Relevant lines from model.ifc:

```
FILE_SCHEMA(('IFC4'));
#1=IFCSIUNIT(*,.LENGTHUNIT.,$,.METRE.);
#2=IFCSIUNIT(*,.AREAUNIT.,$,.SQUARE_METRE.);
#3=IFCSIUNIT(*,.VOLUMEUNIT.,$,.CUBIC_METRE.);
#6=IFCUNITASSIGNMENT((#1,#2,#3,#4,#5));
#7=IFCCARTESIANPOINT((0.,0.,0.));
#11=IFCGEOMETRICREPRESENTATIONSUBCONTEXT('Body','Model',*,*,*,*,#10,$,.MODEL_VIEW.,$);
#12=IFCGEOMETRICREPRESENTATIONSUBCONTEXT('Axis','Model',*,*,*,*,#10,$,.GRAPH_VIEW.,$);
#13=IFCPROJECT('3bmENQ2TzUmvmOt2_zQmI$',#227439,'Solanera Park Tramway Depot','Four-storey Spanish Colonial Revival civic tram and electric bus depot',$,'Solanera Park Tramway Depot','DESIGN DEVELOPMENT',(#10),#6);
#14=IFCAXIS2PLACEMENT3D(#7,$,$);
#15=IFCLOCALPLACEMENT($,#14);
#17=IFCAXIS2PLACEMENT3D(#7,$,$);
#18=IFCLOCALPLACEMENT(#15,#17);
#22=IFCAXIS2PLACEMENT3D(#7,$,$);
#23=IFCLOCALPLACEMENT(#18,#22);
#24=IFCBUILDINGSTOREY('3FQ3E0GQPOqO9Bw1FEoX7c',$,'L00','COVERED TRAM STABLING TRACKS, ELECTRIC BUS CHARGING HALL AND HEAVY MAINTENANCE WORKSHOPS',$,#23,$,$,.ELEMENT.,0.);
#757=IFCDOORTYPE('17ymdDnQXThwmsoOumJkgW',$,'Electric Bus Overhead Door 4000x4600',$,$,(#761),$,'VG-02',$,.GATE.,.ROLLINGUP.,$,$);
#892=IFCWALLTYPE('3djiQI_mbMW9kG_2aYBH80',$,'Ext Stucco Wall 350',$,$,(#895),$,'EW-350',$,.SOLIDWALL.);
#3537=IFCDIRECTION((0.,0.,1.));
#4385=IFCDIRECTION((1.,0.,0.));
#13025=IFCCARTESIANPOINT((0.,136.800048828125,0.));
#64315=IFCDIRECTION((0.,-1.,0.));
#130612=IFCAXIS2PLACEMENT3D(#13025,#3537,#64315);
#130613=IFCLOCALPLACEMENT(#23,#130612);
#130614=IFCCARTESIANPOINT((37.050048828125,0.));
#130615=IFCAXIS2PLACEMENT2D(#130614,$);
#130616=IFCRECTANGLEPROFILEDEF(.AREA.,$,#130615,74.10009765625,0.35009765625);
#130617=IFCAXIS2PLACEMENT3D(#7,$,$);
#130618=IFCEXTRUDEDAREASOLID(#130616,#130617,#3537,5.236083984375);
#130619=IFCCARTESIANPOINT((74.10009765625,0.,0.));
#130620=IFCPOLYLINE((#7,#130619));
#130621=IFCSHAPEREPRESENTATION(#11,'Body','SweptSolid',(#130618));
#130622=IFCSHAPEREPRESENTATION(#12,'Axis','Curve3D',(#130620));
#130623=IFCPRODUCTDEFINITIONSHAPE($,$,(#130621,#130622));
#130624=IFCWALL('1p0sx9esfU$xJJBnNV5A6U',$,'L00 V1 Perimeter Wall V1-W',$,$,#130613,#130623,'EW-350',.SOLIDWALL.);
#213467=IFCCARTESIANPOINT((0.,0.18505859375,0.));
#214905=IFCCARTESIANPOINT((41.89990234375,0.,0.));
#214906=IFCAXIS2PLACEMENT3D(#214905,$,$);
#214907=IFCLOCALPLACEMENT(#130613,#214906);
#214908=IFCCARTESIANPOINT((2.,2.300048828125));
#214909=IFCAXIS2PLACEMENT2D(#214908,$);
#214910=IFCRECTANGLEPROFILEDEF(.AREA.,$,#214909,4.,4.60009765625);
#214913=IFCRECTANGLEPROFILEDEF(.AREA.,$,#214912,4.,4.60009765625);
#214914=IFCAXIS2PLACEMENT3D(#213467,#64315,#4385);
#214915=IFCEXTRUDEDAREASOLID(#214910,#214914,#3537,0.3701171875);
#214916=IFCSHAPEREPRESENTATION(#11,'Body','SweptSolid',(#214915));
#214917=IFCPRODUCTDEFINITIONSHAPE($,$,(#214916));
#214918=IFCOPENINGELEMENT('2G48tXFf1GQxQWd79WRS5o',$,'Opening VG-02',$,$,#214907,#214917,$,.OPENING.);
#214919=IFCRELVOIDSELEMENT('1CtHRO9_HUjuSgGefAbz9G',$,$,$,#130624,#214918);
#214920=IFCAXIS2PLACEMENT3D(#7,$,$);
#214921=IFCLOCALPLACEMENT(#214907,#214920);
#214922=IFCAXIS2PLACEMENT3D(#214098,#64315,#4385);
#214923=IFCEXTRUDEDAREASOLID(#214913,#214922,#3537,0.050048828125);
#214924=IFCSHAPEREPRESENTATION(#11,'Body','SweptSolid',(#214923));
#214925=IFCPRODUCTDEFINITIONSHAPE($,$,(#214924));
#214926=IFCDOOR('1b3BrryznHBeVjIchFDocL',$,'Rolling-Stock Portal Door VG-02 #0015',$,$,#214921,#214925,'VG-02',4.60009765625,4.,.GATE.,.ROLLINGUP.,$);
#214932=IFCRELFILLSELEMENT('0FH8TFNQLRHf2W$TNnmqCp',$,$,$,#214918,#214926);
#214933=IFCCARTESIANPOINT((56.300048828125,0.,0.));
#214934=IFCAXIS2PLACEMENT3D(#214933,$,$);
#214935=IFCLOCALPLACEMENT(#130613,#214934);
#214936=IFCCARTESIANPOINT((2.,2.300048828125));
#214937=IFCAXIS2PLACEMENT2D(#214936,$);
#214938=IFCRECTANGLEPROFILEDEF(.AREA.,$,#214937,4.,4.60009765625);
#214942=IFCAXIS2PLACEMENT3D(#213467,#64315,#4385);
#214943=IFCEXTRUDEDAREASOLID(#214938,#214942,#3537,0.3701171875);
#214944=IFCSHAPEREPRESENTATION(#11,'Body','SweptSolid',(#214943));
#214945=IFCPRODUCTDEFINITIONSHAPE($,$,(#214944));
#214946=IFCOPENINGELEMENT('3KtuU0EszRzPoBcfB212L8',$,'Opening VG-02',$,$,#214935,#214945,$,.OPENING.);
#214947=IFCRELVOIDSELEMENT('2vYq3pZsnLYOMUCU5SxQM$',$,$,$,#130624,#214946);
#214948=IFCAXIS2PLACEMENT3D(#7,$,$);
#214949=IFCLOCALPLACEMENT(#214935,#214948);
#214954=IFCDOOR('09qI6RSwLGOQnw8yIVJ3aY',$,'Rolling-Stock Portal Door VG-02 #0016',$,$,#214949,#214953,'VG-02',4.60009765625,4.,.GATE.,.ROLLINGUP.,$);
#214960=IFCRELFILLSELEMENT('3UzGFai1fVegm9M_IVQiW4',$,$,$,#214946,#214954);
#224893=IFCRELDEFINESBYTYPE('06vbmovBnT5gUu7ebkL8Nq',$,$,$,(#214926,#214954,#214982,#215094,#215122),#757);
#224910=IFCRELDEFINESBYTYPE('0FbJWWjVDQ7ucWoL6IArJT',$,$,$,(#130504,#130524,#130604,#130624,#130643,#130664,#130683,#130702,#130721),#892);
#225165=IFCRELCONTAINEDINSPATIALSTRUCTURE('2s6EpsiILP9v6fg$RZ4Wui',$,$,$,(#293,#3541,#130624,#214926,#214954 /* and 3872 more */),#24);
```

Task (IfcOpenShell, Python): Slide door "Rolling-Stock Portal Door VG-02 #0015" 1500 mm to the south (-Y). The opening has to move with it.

```python
import ifcopenshell
import ifcopenshell.api.geometry
import ifcopenshell.util.placement
import ifcopenshell.util.unit

model = ifcopenshell.open("model.ifc")
unit_scale = ifcopenshell.util.unit.calculate_unit_scale(model)

door = model.by_guid("1b3BrryznHBeVjIchFDocL")
opening = door.FillsVoids[0].RelatingOpeningElement
wall = opening.VoidsElements[0].RelatingBuildingElement

wall_matrix = ifcopenshell.util.placement.get_local_placement(wall.ObjectPlacement)
shift = wall_matrix[:3, 0] * 1.5 / unit_scale
before = ifcopenshell.util.placement.get_local_placement(door.ObjectPlacement)[:3, 3].copy()

# The door is placed relative to its opening, so it follows when the opening moves.
matrix = ifcopenshell.util.placement.get_local_placement(opening.ObjectPlacement)
matrix[:3, 3] += shift
ifcopenshell.api.geometry.edit_object_placement(
    model, product=opening, matrix=matrix, is_si=False, should_transform_children=True
)

after = ifcopenshell.util.placement.get_local_placement(door.ObjectPlacement)[:3, 3]
print("door moved by", (after - before).round(3) + 0.0)

model.write("model_edited.ifc")
```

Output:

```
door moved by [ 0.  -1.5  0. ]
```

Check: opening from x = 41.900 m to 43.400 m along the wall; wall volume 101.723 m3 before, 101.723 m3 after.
